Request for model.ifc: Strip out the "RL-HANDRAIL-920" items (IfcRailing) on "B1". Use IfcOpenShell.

First a look at what the model holds.

```python
import ifcopenshell
import ifcopenshell.util.element

model = ifcopenshell.open("model.ifc")
print(model.schema)
storey = next(s for s in model.by_type("IfcBuildingStorey") if s.Name == "B1")
railings = [e for e in ifcopenshell.util.element.get_decomposition(storey) if e.is_a("IfcRailing")]
seen = {}
for e in railings:
    element_type = ifcopenshell.util.element.get_type(e)
    name = element_type.Name if element_type not in (None, e) else None
    seen[name] = seen.get(name, 0) + 1
for name, count in sorted(seen.items(), key=str):
    print(count, "x", name)
```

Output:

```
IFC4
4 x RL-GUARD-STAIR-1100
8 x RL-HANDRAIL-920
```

```python
import ifcopenshell
import ifcopenshell.api.root
import ifcopenshell.util.element

model = ifcopenshell.open("model.ifc")

storey = next(s for s in model.by_type("IfcBuildingStorey") if s.Name == "B1")
railings = [e for e in ifcopenshell.util.element.get_decomposition(storey) if e.is_a("IfcRailing")]
targets = [e for e in railings if (t := ifcopenshell.util.element.get_type(e)) not in (None, e) and t.Name == "RL-HANDRAIL-920"]

for e in targets:
    ifcopenshell.api.root.remove_product(model, product=e)
print(len(targets), "removed")

model.write("model_edited.ifc")
```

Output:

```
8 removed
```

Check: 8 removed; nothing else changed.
